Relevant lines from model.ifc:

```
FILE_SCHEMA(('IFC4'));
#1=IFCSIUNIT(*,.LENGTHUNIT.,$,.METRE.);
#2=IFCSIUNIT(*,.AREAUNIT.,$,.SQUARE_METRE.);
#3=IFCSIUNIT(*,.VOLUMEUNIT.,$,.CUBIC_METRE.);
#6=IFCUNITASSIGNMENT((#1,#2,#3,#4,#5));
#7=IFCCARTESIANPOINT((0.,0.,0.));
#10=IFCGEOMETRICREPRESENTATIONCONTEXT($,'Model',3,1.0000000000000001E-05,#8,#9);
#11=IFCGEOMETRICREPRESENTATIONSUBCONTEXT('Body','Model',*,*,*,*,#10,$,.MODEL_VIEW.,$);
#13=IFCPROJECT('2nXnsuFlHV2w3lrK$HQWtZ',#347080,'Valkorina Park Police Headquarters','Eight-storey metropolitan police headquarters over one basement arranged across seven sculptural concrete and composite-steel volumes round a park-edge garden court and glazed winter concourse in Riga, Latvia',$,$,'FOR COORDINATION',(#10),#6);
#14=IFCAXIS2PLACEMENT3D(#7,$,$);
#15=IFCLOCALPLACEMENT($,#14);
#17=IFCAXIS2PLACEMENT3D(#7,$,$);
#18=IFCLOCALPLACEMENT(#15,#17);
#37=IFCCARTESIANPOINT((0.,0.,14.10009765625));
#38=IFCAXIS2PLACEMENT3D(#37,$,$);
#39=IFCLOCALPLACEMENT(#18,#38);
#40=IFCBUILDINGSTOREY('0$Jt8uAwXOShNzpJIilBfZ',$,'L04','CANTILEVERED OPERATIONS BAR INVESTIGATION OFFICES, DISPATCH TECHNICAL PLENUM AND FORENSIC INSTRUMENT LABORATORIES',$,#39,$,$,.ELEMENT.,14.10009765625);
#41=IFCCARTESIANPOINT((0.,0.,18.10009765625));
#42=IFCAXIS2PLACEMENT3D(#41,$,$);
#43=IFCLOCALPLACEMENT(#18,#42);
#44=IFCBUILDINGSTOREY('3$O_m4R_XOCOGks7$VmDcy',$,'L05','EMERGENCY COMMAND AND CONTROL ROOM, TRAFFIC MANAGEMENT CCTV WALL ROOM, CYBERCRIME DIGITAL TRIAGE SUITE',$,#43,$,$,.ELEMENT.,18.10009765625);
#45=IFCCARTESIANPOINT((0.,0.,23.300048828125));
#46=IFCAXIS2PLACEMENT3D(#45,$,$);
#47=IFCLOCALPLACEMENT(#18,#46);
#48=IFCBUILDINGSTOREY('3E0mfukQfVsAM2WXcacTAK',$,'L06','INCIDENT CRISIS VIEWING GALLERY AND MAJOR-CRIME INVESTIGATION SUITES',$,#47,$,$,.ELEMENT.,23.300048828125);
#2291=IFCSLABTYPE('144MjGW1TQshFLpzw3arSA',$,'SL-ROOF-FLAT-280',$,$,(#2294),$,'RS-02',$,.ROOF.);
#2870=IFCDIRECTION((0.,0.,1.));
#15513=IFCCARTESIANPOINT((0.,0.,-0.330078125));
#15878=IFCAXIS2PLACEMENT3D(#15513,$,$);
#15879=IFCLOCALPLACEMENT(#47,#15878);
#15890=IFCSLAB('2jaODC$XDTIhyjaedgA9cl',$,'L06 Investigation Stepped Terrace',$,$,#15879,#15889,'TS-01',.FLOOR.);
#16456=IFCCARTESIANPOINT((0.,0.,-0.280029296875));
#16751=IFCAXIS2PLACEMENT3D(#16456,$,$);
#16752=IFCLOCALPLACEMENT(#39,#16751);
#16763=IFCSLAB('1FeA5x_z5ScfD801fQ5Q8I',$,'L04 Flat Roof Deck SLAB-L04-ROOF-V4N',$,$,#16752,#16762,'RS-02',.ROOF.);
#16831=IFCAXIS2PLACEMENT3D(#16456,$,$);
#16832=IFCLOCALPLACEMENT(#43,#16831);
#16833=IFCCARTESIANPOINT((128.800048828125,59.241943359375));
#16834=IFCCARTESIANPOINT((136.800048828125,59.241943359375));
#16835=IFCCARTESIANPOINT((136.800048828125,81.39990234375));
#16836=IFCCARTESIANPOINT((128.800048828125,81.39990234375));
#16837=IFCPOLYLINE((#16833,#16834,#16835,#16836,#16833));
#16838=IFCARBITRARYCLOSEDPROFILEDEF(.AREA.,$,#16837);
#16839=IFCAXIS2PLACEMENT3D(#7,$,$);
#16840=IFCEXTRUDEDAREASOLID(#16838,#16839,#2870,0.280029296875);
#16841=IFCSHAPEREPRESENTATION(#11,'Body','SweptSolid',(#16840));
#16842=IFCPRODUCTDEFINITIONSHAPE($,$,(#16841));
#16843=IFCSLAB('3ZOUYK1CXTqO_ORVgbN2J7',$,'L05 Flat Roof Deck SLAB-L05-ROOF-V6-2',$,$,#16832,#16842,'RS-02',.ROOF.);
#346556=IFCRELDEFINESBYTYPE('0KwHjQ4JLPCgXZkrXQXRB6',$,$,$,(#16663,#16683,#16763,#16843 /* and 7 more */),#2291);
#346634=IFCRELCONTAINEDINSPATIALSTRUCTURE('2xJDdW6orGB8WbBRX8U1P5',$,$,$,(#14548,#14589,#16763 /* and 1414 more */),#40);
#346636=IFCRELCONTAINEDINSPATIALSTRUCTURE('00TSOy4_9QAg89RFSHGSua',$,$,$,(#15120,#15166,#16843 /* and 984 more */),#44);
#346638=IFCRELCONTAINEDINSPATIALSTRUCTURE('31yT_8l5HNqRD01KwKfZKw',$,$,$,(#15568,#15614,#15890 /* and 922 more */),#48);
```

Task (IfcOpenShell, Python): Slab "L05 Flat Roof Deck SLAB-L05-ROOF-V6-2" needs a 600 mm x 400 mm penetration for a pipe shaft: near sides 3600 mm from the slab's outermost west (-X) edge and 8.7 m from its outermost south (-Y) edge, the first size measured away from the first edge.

```python
import numpy as np
import ifcopenshell
import ifcopenshell.api.feature
import ifcopenshell.api.geometry
import ifcopenshell.api.root
import ifcopenshell.geom
import ifcopenshell.util.placement
import ifcopenshell.util.representation
import ifcopenshell.util.shape
import ifcopenshell.util.unit

model = ifcopenshell.open("model.ifc")
unit_scale = ifcopenshell.util.unit.calculate_unit_scale(model)
settings = ifcopenshell.geom.settings()


def volume(element):
    """Net volume in cubic metres, openings subtracted."""
    shape = ifcopenshell.geom.create_shape(settings, element)
    return ifcopenshell.util.shape.get_volume(shape.geometry)


slab = model.by_guid("3ZOUYK1CXTqO_ORVgbN2J7")
before = volume(slab)

# Extent in the slab's own axes, in metres. The edges named are its -X and -Y sides.
slab_shape = ifcopenshell.geom.create_shape(settings, slab)
vertices = ifcopenshell.util.shape.get_vertices(slab_shape.geometry)
x_min, y_min, bottom = vertices.min(axis=0)
top = vertices[:, 2].max()

opening = ifcopenshell.api.root.create_entity(model, ifc_class="IfcOpeningElement", name="Pipe shaft opening", predefined_type="OPENING")
context = ifcopenshell.util.representation.get_context(model, "Model", "Body", "MODEL_VIEW")
width, depth = 0.6, 0.4
outline = [(0.0, 0.0), (width, 0.0), (width, depth), (0.0, depth), (0.0, 0.0)]
# Overshoot both faces by 50 mm so the cut is clean.
shape = ifcopenshell.api.geometry.add_slab_representation(
    model, context=context, depth=top - bottom + 0.1, polyline=outline
)
ifcopenshell.api.geometry.assign_representation(model, product=opening, representation=shape)

matrix = ifcopenshell.util.placement.get_local_placement(slab.ObjectPlacement)
matrix[:, 3] = matrix @ np.append(np.array([x_min + 3.6, y_min + 8.7, bottom - 0.05]) / unit_scale, 1.0)
ifcopenshell.api.geometry.edit_object_placement(model, product=opening, matrix=matrix, is_si=False)
ifcopenshell.api.feature.add_feature(model, feature=opening, element=slab)

after = volume(slab)

print(f"slab volume {before:.3f} -> {after:.3f} m3")

model.write("model_rev.ifc")
```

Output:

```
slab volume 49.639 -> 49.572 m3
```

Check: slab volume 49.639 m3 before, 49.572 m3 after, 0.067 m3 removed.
